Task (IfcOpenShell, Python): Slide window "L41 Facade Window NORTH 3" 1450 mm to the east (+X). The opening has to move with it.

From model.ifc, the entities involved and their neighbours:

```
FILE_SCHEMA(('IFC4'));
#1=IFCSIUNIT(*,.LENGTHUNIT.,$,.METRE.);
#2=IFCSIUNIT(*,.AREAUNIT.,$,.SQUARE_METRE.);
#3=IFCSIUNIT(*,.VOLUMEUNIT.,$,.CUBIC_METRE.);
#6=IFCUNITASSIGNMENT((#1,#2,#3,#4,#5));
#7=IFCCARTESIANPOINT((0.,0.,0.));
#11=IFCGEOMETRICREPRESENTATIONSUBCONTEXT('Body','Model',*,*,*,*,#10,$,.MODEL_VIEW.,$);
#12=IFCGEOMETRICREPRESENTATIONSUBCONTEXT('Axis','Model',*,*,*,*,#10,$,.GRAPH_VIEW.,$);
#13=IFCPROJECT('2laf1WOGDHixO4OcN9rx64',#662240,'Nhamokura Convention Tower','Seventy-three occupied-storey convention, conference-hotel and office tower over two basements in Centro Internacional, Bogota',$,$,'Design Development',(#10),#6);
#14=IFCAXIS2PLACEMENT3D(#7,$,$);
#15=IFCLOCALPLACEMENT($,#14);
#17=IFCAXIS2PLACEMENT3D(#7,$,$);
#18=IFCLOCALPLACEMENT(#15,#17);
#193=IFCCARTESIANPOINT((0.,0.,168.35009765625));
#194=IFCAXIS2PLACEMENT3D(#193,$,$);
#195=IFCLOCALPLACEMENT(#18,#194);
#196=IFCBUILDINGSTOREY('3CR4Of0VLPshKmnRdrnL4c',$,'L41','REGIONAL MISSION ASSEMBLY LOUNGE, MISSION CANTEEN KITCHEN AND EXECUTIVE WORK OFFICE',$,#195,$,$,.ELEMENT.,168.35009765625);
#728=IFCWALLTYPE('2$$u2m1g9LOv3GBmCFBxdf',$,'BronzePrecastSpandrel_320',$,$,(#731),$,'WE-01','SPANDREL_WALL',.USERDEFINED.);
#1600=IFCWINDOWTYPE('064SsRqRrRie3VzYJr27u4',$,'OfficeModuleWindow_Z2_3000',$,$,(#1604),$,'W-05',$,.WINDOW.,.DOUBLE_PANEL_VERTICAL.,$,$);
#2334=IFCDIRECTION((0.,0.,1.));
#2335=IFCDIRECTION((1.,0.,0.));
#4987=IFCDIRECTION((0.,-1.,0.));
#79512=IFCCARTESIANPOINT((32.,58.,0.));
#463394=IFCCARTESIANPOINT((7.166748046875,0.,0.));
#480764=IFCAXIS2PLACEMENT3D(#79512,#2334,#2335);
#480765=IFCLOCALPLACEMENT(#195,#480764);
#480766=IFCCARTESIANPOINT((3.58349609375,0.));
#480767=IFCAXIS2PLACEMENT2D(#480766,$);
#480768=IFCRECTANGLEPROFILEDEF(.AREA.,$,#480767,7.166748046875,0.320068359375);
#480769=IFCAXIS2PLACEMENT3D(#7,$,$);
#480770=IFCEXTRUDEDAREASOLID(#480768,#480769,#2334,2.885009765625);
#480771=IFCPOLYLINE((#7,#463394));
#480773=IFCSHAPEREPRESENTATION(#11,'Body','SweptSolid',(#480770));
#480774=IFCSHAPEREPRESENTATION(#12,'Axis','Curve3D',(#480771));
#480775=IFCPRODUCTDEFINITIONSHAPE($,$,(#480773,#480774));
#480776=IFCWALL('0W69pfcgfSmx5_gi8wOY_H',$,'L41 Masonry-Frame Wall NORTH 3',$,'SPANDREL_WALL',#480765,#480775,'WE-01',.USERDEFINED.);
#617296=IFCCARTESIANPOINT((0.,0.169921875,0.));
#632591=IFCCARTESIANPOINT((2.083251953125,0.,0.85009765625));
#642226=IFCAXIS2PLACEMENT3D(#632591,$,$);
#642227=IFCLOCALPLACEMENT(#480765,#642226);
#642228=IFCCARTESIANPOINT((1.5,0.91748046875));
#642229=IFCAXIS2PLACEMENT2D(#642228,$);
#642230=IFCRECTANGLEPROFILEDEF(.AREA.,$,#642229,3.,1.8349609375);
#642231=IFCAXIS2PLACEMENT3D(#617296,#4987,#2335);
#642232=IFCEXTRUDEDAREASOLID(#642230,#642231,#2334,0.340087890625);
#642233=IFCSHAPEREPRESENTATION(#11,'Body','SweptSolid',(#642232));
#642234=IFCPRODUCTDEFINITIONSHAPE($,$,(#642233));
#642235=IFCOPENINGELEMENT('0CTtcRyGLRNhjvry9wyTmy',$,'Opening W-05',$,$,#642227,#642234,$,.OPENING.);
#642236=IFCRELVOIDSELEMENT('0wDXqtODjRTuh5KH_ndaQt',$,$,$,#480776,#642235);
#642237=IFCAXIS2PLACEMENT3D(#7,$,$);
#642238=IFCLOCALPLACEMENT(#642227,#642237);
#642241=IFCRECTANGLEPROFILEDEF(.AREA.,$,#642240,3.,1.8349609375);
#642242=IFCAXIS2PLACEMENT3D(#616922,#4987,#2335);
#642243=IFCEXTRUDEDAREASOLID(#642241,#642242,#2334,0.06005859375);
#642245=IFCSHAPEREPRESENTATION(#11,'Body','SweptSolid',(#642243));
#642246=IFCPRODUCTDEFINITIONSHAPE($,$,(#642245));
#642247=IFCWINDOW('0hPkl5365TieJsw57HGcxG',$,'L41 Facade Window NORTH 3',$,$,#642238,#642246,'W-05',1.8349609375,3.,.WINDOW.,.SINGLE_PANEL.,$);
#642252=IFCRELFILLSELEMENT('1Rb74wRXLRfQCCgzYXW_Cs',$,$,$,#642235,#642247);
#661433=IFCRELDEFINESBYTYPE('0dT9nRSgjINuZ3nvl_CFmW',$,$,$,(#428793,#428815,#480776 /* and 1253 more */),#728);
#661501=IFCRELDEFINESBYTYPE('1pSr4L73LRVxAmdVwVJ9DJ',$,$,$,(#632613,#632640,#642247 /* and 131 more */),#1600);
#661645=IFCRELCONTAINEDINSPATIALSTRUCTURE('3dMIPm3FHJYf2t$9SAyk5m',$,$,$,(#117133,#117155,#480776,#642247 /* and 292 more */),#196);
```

```python
import ifcopenshell
import ifcopenshell.api.geometry
import ifcopenshell.util.placement

model = ifcopenshell.open("model.ifc")

window = model.by_guid("0hPkl5365TieJsw57HGcxG")
opening = window.FillsVoids[0].RelatingOpeningElement
wall = opening.VoidsElements[0].RelatingBuildingElement

wall_matrix = ifcopenshell.util.placement.get_local_placement(wall.ObjectPlacement)
shift = wall_matrix[:3, 0] * 1.45
before = ifcopenshell.util.placement.get_local_placement(window.ObjectPlacement)[:3, 3].copy()

# The window is placed relative to its opening, so it follows when the opening moves.
matrix = ifcopenshell.util.placement.get_local_placement(opening.ObjectPlacement)
matrix[:3, 3] += shift
ifcopenshell.api.geometry.edit_object_placement(
    model, product=opening, matrix=matrix, is_si=False, should_transform_children=True
)

after = ifcopenshell.util.placement.get_local_placement(window.ObjectPlacement)[:3, 3]
print("window moved by", (after - before).round(3) + 0.0)

model.write("model_v2.ifc")
```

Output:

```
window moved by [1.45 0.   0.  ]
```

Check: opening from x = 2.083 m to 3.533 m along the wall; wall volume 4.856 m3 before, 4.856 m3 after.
